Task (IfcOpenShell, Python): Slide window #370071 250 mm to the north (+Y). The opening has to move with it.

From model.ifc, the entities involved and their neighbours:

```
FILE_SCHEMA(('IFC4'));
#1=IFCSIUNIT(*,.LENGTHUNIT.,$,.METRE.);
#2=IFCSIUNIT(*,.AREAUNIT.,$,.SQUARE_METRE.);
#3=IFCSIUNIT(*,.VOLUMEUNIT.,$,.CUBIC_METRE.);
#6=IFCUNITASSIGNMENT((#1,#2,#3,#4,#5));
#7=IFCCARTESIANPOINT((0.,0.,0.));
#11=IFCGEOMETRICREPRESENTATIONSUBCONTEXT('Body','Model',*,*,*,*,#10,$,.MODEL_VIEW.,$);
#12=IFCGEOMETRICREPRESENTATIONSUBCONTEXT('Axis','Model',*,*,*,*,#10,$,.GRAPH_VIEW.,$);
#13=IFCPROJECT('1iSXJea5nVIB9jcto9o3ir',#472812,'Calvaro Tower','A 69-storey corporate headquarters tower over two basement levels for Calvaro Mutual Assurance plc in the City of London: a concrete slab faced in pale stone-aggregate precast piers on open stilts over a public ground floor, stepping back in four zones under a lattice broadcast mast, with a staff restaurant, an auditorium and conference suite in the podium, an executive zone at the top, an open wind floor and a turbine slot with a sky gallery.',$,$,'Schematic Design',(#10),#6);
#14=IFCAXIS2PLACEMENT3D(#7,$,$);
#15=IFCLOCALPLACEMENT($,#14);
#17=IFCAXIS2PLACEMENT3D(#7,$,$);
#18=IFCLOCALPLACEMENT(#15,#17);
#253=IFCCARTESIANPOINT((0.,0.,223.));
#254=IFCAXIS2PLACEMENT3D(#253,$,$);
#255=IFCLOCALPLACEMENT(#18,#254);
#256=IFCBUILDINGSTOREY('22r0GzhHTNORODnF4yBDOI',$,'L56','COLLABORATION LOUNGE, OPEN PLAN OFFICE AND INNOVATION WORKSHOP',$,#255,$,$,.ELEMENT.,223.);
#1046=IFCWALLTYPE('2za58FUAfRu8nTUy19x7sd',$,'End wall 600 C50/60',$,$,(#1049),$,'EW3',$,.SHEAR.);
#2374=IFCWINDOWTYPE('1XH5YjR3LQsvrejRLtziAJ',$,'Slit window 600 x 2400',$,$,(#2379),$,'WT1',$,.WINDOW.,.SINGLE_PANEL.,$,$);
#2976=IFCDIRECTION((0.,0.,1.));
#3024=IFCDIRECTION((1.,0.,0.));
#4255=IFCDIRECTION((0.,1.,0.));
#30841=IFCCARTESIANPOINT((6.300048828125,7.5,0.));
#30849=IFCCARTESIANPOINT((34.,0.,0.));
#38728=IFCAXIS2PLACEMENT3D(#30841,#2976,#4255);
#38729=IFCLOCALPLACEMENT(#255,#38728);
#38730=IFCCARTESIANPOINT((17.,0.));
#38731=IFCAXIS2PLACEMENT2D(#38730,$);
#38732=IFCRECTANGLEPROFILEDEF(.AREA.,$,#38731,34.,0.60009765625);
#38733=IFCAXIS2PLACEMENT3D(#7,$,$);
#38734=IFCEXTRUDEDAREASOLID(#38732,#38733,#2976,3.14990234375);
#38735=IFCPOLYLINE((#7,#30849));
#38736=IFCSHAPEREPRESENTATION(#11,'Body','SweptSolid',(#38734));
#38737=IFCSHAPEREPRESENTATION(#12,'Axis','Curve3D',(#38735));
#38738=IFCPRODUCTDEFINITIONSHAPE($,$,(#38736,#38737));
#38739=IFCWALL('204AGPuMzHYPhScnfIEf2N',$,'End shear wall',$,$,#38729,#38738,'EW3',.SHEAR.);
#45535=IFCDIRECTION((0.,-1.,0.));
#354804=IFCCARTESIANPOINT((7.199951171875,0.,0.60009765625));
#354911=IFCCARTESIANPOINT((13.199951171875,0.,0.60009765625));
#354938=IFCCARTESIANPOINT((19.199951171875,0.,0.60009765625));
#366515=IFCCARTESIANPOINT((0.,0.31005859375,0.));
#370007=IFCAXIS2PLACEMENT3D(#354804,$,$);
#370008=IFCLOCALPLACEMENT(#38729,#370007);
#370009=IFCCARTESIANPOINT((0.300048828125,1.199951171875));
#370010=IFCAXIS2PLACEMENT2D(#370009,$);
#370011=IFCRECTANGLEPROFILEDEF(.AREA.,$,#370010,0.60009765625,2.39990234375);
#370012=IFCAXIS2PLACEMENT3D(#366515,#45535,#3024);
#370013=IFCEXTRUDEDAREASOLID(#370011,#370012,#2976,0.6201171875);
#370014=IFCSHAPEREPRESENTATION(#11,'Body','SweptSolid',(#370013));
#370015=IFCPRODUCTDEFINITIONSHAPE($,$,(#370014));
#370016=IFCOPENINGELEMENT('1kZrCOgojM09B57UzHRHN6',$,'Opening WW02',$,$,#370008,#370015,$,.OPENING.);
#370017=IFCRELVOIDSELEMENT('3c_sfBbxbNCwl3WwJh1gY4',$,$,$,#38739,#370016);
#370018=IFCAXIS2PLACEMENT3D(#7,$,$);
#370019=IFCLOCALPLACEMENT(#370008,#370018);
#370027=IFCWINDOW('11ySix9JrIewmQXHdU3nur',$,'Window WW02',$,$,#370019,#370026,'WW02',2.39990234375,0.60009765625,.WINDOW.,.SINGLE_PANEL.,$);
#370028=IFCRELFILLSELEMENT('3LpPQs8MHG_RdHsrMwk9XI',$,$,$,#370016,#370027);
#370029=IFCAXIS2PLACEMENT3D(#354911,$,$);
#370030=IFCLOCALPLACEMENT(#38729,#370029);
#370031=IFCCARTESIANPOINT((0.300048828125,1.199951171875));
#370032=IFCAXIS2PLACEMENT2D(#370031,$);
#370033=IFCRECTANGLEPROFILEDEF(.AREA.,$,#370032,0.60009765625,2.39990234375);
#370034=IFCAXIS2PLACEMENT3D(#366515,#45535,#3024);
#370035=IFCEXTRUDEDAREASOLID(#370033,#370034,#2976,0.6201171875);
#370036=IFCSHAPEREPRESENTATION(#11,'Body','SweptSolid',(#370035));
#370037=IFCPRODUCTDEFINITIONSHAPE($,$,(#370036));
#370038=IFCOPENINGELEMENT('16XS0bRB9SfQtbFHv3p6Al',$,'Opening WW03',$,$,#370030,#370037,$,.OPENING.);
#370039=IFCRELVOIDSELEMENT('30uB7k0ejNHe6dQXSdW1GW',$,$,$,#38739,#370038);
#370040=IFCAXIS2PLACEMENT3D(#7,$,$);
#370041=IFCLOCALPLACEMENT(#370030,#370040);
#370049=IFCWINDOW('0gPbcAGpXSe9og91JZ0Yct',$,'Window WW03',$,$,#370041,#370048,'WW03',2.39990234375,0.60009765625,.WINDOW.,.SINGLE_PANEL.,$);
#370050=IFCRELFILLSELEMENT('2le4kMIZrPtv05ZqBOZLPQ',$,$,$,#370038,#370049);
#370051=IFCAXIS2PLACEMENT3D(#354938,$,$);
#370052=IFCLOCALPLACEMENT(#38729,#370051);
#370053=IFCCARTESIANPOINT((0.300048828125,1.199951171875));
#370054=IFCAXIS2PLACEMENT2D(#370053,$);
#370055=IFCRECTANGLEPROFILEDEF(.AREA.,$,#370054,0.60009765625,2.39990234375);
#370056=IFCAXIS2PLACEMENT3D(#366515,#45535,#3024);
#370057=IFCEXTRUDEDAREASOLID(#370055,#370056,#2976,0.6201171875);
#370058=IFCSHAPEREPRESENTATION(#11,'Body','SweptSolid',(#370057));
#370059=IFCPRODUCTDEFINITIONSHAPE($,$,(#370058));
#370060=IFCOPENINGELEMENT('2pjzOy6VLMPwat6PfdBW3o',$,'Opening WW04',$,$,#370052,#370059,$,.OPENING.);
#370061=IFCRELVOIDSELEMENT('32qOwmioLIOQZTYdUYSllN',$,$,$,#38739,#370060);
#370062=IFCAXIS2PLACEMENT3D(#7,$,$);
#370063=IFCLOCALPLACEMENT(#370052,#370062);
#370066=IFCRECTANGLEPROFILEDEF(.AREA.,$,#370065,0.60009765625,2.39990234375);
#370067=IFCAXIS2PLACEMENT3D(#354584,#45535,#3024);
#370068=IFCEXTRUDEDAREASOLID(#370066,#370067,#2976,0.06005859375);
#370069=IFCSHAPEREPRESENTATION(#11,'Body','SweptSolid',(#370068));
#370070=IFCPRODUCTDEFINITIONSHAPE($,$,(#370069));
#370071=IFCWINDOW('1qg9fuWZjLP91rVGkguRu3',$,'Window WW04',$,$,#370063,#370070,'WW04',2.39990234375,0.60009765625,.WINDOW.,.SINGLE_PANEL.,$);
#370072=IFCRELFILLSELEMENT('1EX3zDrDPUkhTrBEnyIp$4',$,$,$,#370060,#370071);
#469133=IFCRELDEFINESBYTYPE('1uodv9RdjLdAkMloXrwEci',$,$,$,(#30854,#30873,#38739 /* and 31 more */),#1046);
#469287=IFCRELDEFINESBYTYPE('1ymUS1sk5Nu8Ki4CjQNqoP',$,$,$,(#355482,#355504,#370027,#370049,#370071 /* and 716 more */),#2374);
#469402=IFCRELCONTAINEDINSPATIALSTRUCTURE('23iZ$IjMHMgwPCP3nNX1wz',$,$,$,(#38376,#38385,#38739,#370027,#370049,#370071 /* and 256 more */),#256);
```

```python
import ifcopenshell
import ifcopenshell.api.geometry
import ifcopenshell.util.placement

model = ifcopenshell.open("model.ifc")

window = model.by_guid("1qg9fuWZjLP91rVGkguRu3")
opening = window.FillsVoids[0].RelatingOpeningElement
wall = opening.VoidsElements[0].RelatingBuildingElement

wall_matrix = ifcopenshell.util.placement.get_local_placement(wall.ObjectPlacement)
shift = wall_matrix[:3, 0] * 0.25
before = ifcopenshell.util.placement.get_local_placement(window.ObjectPlacement)[:3, 3].copy()

# The window is placed relative to its opening, so it follows when the opening moves.
matrix = ifcopenshell.util.placement.get_local_placement(opening.ObjectPlacement)
matrix[:3, 3] += shift
ifcopenshell.api.geometry.edit_object_placement(
    model, product=opening, matrix=matrix, is_si=False, should_transform_children=True
)

after = ifcopenshell.util.placement.get_local_placement(window.ObjectPlacement)[:3, 3]
print("window moved by", (after - before).round(3) + 0.0)

model.write("model_edited.ifc")
```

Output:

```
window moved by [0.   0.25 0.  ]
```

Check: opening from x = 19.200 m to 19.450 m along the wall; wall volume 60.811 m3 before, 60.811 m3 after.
